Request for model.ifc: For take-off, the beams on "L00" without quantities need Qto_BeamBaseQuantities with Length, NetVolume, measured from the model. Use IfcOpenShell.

First a look at what the model holds.

```python
import ifcopenshell
import ifcopenshell.util.element
import ifcopenshell.util.unit

model = ifcopenshell.open("model.ifc")
print(model.schema)
for unit_type in ("LENGTHUNIT", "AREAUNIT", "VOLUMEUNIT"):
    print(unit_type, ifcopenshell.util.unit.calculate_unit_scale(model, unit_type))
storey = next(s for s in model.by_type("IfcBuildingStorey") if s.Name == "L00")
beams = [e for e in ifcopenshell.util.element.get_decomposition(storey) if e.is_a("IfcBeam")]
for e in sorted(beams, key=lambda e: e.id()):
    print(e.id(), e.is_a(), e.Name, list(ifcopenshell.util.element.get_psets(e, qtos_only=True)), sep=" | ")
```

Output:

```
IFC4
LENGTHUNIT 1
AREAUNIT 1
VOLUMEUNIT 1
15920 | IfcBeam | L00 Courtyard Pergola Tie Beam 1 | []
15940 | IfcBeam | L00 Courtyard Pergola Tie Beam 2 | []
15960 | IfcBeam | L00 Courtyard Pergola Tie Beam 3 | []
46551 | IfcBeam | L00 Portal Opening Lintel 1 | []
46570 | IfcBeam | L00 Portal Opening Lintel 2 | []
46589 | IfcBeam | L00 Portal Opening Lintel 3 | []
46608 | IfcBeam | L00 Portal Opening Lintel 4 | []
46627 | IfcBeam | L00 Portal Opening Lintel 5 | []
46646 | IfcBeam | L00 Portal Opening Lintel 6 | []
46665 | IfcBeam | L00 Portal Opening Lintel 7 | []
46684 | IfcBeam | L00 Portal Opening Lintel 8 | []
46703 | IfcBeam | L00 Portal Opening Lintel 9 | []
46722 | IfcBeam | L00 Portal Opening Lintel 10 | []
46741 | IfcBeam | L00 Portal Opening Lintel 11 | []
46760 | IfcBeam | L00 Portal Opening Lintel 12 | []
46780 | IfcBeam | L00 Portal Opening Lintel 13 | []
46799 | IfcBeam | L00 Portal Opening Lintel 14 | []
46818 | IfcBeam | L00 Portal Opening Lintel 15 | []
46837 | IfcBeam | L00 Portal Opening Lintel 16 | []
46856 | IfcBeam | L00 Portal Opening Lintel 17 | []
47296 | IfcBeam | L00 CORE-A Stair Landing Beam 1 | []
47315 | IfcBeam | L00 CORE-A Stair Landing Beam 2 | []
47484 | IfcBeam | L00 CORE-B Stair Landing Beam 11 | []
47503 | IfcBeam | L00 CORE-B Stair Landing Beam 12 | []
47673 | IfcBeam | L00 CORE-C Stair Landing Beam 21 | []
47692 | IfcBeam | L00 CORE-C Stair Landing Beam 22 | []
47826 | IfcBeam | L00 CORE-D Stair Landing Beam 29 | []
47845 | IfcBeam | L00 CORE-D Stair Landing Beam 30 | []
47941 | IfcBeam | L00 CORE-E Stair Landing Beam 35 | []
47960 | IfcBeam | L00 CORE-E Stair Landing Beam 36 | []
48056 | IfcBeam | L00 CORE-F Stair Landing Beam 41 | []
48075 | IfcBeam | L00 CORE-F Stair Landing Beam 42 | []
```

```python
import ifcopenshell
import ifcopenshell.api.pset
import ifcopenshell.geom
import ifcopenshell.util.element
import ifcopenshell.util.shape
import ifcopenshell.util.unit

model = ifcopenshell.open("model.ifc")
unit_scale = ifcopenshell.util.unit.calculate_unit_scale(model)
volume_scale = ifcopenshell.util.unit.calculate_unit_scale(model, "VOLUMEUNIT")
settings = ifcopenshell.geom.settings()

storey = next(s for s in model.by_type("IfcBuildingStorey") if s.Name == "L00")
beams = [e for e in ifcopenshell.util.element.get_decomposition(storey) if e.is_a("IfcBeam")]

for e in sorted(beams, key=lambda e: e.id()):
    if ifcopenshell.util.element.get_psets(e, qtos_only=True, should_inherit=False):
        continue
    # Geometry comes back in metres, in the element's own axes.
    shape = ifcopenshell.geom.create_shape(settings, e)
    values = {
        "Length": ifcopenshell.util.shape.get_max_xyz(shape.geometry) / unit_scale,
        "NetVolume": ifcopenshell.util.shape.get_volume(shape.geometry) / volume_scale,
    }
    qto = ifcopenshell.api.pset.add_qto(model, product=e, name="Qto_BeamBaseQuantities")
    ifcopenshell.api.pset.edit_qto(model, qto=qto, properties=values)
    print(e.id(), {k: round(v, 3) for k, v in values.items()})

model.write("model_updated.ifc")
```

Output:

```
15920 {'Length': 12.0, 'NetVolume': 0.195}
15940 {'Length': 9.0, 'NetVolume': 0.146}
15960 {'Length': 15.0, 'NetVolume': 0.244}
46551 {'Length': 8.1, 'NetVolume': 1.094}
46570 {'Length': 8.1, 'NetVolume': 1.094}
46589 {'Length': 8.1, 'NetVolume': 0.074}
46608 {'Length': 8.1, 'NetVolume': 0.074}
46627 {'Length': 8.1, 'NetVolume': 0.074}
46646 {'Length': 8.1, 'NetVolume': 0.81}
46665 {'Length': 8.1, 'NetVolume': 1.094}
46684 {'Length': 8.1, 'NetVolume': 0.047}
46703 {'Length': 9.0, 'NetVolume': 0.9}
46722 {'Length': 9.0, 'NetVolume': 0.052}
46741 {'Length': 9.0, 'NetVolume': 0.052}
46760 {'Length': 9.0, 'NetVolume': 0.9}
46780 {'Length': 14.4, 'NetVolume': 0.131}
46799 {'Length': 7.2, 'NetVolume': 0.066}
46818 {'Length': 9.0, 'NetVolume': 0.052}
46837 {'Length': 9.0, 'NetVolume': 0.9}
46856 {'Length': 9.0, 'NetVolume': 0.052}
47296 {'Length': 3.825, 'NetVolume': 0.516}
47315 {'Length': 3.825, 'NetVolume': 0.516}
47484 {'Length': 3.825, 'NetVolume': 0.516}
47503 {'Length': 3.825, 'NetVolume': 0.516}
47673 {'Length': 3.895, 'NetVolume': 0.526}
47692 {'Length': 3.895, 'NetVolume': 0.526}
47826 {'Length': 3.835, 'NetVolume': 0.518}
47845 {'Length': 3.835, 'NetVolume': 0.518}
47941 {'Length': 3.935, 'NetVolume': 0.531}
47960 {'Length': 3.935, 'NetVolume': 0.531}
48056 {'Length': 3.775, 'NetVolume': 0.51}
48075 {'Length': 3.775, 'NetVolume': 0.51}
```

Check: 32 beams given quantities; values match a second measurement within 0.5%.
